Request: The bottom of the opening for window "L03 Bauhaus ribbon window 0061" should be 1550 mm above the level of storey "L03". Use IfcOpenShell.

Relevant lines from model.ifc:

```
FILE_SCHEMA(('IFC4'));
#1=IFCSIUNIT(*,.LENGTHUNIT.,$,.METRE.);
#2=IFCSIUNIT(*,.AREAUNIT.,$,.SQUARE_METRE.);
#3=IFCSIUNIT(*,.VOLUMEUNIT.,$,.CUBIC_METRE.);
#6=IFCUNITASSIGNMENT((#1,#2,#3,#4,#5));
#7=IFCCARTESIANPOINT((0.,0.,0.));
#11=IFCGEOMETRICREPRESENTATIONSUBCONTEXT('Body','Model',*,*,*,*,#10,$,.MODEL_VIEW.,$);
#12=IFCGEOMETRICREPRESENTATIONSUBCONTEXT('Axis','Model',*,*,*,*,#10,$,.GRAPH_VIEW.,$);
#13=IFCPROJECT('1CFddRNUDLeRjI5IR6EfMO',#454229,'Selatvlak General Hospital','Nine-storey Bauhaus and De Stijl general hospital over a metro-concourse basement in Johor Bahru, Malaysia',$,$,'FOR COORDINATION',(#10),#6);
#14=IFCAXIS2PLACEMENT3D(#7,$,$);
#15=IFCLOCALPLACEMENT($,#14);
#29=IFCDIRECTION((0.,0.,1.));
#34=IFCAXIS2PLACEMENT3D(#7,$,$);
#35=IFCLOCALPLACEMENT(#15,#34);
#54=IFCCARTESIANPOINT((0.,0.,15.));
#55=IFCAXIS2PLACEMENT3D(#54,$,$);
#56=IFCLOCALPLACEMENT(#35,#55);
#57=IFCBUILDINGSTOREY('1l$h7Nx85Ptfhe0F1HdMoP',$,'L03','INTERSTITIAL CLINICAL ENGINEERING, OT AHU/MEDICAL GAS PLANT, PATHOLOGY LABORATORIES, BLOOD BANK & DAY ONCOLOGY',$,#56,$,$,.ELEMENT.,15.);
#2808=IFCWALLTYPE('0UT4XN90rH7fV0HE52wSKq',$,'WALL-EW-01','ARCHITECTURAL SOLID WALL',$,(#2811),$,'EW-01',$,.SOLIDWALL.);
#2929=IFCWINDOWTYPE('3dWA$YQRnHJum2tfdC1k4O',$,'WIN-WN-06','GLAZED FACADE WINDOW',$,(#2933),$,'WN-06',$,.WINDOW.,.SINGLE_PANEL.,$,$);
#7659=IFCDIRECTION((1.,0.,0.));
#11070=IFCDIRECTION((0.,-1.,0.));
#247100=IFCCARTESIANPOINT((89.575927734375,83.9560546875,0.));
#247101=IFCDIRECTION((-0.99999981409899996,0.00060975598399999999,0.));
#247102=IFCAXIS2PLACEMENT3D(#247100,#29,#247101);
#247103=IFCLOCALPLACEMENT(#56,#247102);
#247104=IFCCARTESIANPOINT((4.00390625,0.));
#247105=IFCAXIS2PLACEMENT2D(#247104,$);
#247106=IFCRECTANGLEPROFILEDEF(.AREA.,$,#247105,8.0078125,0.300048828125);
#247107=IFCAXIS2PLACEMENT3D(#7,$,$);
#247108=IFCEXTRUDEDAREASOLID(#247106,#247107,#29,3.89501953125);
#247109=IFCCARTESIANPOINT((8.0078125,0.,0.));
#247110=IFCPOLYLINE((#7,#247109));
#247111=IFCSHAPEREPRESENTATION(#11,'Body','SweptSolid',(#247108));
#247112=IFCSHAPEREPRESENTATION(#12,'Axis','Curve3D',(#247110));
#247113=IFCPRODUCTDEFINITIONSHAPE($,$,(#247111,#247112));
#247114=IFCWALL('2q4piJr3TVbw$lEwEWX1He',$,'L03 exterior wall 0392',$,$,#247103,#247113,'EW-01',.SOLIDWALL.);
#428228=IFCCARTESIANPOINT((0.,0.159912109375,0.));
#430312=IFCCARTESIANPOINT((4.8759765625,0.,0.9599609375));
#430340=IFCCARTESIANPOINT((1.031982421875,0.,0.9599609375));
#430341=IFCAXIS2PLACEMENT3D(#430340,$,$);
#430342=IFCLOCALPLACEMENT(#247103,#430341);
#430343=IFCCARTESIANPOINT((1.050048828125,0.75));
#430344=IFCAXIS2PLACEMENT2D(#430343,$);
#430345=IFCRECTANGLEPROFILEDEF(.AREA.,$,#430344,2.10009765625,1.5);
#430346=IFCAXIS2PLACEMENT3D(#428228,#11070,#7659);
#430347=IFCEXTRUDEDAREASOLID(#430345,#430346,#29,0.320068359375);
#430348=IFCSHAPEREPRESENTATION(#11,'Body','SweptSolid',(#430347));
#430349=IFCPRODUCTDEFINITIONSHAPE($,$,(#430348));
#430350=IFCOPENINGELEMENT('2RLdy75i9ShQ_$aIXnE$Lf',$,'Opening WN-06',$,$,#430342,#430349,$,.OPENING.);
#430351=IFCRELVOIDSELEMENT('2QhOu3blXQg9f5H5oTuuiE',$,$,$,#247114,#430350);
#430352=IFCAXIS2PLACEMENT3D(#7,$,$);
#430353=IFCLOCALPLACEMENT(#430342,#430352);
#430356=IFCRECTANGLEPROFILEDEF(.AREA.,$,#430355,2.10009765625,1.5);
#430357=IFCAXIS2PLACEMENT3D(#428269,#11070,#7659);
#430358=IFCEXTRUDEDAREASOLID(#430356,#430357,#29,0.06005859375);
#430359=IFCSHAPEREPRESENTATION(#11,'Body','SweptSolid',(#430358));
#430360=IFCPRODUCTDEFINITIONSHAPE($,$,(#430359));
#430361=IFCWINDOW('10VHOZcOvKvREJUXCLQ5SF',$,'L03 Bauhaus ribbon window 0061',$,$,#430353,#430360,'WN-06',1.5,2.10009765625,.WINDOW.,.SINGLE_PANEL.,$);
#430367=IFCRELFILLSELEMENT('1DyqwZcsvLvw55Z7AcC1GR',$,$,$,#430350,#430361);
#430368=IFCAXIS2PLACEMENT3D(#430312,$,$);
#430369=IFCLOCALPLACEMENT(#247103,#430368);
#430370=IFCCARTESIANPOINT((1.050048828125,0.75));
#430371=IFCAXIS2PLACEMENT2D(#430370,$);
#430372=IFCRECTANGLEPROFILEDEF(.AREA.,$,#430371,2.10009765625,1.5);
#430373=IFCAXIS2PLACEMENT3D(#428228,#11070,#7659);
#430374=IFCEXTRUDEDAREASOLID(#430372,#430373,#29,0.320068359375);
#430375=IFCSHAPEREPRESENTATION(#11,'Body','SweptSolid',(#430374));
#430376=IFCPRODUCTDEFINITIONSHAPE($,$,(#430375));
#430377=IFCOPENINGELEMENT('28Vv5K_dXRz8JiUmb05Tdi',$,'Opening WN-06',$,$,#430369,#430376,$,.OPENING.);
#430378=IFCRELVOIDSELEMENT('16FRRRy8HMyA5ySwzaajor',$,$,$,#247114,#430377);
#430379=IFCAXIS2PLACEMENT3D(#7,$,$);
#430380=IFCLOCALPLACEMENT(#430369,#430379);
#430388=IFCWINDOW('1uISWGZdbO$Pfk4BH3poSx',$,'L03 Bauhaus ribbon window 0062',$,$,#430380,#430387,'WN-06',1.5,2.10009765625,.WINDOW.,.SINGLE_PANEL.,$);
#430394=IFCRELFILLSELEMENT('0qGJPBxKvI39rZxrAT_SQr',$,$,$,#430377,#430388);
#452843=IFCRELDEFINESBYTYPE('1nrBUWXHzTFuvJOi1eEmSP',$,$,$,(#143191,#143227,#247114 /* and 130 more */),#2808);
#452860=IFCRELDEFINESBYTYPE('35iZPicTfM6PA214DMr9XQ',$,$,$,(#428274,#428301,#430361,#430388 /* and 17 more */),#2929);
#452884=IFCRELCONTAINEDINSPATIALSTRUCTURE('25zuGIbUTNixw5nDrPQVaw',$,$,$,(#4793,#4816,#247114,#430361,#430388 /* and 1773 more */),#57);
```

```python
import numpy as np
import ifcopenshell
import ifcopenshell.api.geometry
import ifcopenshell.geom
import ifcopenshell.util.element
import ifcopenshell.util.placement
import ifcopenshell.util.shape
import ifcopenshell.util.unit

model = ifcopenshell.open("model.ifc")
unit_scale = ifcopenshell.util.unit.calculate_unit_scale(model)

window = model.by_guid("10VHOZcOvKvREJUXCLQ5SF")
opening = window.FillsVoids[0].RelatingOpeningElement
storey = ifcopenshell.util.element.get_container(window, ifc_class="IfcBuildingStorey")
level = ifcopenshell.util.placement.get_local_placement(storey.ObjectPlacement)[2, 3]

# The opening's origin need not be at the sill, so measure its lowest point.
shape = ifcopenshell.geom.create_shape(ifcopenshell.geom.settings(), opening)
bottom = ifcopenshell.util.shape.get_shape_bottom_elevation(shape, shape.geometry) / unit_scale
dz = level + 1.55 - bottom

shift = np.array([0.0, 0.0, dz])
# The window is placed relative to its opening, so it follows when the opening moves.
matrix = ifcopenshell.util.placement.get_local_placement(opening.ObjectPlacement)
matrix[:3, 3] += shift
ifcopenshell.api.geometry.edit_object_placement(
    model, product=opening, matrix=matrix, is_si=False, should_transform_children=True
)

print(f"moved by {dz * unit_scale:+.3f} m")

model.write("model_v2.ifc")
```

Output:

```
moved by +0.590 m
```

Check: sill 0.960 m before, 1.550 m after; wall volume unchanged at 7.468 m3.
